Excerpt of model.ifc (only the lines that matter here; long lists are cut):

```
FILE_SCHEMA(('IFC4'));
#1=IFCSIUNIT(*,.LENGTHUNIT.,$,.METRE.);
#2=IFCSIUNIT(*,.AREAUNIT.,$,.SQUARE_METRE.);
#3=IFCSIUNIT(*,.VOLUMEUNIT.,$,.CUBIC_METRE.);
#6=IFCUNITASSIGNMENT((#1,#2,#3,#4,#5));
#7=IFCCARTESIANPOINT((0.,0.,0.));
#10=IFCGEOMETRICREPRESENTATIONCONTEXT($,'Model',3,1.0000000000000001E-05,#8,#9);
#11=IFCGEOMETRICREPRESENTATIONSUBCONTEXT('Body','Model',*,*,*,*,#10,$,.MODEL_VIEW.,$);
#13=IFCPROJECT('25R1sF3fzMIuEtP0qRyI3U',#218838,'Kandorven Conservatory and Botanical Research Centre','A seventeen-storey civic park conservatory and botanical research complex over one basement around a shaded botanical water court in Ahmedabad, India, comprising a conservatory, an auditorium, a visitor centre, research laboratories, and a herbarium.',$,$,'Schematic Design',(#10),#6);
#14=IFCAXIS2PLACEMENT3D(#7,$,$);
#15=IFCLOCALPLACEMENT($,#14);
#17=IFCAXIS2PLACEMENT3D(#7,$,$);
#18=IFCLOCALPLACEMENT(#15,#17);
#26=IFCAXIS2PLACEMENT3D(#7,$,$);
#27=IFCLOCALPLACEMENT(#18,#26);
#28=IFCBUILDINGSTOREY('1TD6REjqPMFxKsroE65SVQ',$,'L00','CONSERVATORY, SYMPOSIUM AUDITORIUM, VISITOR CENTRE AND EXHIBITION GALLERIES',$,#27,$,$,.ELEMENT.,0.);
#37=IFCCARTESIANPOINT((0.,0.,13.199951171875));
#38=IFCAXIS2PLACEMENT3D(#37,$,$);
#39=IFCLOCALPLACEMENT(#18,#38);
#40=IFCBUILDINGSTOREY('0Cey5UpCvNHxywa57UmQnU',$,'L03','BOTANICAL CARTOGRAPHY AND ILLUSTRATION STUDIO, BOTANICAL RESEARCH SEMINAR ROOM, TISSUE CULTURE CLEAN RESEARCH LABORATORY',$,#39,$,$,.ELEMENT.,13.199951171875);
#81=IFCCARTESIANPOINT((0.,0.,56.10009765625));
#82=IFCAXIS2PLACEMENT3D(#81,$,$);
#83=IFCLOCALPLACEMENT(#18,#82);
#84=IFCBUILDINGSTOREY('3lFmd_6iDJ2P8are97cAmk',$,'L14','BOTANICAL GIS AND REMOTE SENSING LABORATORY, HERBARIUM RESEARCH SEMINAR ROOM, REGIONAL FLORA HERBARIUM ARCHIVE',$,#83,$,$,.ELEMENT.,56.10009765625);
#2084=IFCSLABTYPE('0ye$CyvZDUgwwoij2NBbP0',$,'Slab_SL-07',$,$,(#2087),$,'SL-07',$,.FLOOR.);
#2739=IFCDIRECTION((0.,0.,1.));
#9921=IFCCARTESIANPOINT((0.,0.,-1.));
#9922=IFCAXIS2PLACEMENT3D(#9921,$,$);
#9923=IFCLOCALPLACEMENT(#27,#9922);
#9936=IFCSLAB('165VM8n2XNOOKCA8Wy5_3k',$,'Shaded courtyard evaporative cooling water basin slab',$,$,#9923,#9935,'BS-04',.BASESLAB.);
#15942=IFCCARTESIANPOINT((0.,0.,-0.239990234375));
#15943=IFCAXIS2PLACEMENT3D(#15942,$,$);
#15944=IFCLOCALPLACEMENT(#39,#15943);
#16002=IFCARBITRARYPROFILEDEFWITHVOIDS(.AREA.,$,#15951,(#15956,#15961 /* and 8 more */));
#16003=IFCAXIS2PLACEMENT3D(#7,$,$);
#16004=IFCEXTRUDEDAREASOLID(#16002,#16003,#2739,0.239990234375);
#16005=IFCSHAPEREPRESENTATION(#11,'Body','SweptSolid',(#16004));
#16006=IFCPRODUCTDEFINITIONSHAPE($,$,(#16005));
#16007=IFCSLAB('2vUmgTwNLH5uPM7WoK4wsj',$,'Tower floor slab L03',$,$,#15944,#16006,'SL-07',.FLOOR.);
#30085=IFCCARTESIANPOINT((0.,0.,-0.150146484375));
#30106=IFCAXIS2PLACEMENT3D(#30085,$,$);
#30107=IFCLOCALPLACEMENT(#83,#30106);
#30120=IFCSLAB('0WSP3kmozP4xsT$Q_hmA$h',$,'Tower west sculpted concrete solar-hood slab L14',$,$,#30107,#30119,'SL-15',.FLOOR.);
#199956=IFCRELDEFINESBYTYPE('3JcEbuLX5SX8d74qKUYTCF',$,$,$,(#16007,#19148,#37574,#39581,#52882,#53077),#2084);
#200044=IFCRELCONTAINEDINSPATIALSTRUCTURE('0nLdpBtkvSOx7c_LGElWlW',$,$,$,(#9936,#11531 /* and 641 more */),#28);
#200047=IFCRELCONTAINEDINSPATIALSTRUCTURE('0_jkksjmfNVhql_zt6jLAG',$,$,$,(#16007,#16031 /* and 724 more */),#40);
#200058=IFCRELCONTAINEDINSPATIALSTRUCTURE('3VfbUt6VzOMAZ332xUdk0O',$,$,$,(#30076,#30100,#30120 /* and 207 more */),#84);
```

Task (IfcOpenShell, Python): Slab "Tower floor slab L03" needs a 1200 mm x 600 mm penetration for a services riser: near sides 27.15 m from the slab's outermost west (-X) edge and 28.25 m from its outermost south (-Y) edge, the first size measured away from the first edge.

```python
import numpy as np
import ifcopenshell
import ifcopenshell.api.feature
import ifcopenshell.api.geometry
import ifcopenshell.api.root
import ifcopenshell.geom
import ifcopenshell.util.placement
import ifcopenshell.util.representation
import ifcopenshell.util.shape
import ifcopenshell.util.unit

model = ifcopenshell.open("model.ifc")
unit_scale = ifcopenshell.util.unit.calculate_unit_scale(model)
settings = ifcopenshell.geom.settings()


def volume(element):
    """Net volume in cubic metres, openings subtracted."""
    shape = ifcopenshell.geom.create_shape(settings, element)
    return ifcopenshell.util.shape.get_volume(shape.geometry)


slab = model.by_guid("2vUmgTwNLH5uPM7WoK4wsj")
before = volume(slab)

# Extent in the slab's own axes, in metres. The edges named are its -X and -Y sides.
slab_shape = ifcopenshell.geom.create_shape(settings, slab)
vertices = ifcopenshell.util.shape.get_vertices(slab_shape.geometry)
x_min, y_min, bottom = vertices.min(axis=0)
top = vertices[:, 2].max()

opening = ifcopenshell.api.root.create_entity(model, ifc_class="IfcOpeningElement", name="Services riser opening", predefined_type="OPENING")
context = ifcopenshell.util.representation.get_context(model, "Model", "Body", "MODEL_VIEW")
width, depth = 1.2, 0.6
outline = [(0.0, 0.0), (width, 0.0), (width, depth), (0.0, depth), (0.0, 0.0)]
# Overshoot both faces by 50 mm so the cut is clean.
shape = ifcopenshell.api.geometry.add_slab_representation(
    model, context=context, depth=top - bottom + 0.1, polyline=outline
)
ifcopenshell.api.geometry.assign_representation(model, product=opening, representation=shape)

matrix = ifcopenshell.util.placement.get_local_placement(slab.ObjectPlacement)
matrix[:, 3] = matrix @ np.append(np.array([x_min + 27.15, y_min + 28.25, bottom - 0.05]) / unit_scale, 1.0)
ifcopenshell.api.geometry.edit_object_placement(model, product=opening, matrix=matrix, is_si=False)
ifcopenshell.api.feature.add_feature(model, feature=opening, element=slab)

after = volume(slab)

print(f"slab volume {before:.3f} -> {after:.3f} m3")

model.write("model_v2.ifc")
```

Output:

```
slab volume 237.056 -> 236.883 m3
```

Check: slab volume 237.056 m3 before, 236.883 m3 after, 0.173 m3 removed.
